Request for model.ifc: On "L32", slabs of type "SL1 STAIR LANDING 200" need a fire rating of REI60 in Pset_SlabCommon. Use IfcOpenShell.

First a look at what the model holds.

```python
import ifcopenshell
import ifcopenshell.util.element

model = ifcopenshell.open("model.ifc")
print(model.schema)
storey = next(s for s in model.by_type("IfcBuildingStorey") if s.Name == "L32")
slabs = [e for e in ifcopenshell.util.element.get_decomposition(storey) if e.is_a("IfcSlab")]
seen = {}
for e in slabs:
    element_type = ifcopenshell.util.element.get_type(e)
    key = (element_type.Name if element_type != e and element_type else None, ifcopenshell.util.element.get_pset(e, "Pset_SlabCommon", "FireRating"))
    seen[key] = seen.get(key, 0) + 1
for (name, value), count in sorted(seen.items(), key=str):
    print(count, "x", name, "|", value)
```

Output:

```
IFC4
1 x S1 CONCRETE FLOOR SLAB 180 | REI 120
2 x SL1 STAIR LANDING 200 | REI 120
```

```python
import ifcopenshell
import ifcopenshell.api.pset
import ifcopenshell.util.element

model = ifcopenshell.open("model.ifc")

storey = next(s for s in model.by_type("IfcBuildingStorey") if s.Name == "L32")
slabs = [e for e in ifcopenshell.util.element.get_decomposition(storey) if e.is_a("IfcSlab")]

count = 0
for e in slabs:
    element_type = ifcopenshell.util.element.get_type(e)
    if element_type in (None, e) or element_type.Name != "SL1 STAIR LANDING 200":
        continue
    found = ifcopenshell.util.element.get_pset(e, "Pset_SlabCommon", should_inherit=False)
    if found:
        pset = model.by_id(found["id"])
        if len(ifcopenshell.util.element.get_elements_by_pset(pset)) > 1:
            pset = ifcopenshell.api.pset.unshare_pset(model, products=[e], pset=pset)[0]
    else:
        pset = ifcopenshell.api.pset.add_pset(model, product=e, name="Pset_SlabCommon")
    ifcopenshell.api.pset.edit_pset(model, pset=pset, properties={"FireRating": "REI60"})
    count += 1

print(count, "slabs updated")

model.write("model_rev.ifc")
```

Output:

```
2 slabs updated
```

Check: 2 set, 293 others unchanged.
